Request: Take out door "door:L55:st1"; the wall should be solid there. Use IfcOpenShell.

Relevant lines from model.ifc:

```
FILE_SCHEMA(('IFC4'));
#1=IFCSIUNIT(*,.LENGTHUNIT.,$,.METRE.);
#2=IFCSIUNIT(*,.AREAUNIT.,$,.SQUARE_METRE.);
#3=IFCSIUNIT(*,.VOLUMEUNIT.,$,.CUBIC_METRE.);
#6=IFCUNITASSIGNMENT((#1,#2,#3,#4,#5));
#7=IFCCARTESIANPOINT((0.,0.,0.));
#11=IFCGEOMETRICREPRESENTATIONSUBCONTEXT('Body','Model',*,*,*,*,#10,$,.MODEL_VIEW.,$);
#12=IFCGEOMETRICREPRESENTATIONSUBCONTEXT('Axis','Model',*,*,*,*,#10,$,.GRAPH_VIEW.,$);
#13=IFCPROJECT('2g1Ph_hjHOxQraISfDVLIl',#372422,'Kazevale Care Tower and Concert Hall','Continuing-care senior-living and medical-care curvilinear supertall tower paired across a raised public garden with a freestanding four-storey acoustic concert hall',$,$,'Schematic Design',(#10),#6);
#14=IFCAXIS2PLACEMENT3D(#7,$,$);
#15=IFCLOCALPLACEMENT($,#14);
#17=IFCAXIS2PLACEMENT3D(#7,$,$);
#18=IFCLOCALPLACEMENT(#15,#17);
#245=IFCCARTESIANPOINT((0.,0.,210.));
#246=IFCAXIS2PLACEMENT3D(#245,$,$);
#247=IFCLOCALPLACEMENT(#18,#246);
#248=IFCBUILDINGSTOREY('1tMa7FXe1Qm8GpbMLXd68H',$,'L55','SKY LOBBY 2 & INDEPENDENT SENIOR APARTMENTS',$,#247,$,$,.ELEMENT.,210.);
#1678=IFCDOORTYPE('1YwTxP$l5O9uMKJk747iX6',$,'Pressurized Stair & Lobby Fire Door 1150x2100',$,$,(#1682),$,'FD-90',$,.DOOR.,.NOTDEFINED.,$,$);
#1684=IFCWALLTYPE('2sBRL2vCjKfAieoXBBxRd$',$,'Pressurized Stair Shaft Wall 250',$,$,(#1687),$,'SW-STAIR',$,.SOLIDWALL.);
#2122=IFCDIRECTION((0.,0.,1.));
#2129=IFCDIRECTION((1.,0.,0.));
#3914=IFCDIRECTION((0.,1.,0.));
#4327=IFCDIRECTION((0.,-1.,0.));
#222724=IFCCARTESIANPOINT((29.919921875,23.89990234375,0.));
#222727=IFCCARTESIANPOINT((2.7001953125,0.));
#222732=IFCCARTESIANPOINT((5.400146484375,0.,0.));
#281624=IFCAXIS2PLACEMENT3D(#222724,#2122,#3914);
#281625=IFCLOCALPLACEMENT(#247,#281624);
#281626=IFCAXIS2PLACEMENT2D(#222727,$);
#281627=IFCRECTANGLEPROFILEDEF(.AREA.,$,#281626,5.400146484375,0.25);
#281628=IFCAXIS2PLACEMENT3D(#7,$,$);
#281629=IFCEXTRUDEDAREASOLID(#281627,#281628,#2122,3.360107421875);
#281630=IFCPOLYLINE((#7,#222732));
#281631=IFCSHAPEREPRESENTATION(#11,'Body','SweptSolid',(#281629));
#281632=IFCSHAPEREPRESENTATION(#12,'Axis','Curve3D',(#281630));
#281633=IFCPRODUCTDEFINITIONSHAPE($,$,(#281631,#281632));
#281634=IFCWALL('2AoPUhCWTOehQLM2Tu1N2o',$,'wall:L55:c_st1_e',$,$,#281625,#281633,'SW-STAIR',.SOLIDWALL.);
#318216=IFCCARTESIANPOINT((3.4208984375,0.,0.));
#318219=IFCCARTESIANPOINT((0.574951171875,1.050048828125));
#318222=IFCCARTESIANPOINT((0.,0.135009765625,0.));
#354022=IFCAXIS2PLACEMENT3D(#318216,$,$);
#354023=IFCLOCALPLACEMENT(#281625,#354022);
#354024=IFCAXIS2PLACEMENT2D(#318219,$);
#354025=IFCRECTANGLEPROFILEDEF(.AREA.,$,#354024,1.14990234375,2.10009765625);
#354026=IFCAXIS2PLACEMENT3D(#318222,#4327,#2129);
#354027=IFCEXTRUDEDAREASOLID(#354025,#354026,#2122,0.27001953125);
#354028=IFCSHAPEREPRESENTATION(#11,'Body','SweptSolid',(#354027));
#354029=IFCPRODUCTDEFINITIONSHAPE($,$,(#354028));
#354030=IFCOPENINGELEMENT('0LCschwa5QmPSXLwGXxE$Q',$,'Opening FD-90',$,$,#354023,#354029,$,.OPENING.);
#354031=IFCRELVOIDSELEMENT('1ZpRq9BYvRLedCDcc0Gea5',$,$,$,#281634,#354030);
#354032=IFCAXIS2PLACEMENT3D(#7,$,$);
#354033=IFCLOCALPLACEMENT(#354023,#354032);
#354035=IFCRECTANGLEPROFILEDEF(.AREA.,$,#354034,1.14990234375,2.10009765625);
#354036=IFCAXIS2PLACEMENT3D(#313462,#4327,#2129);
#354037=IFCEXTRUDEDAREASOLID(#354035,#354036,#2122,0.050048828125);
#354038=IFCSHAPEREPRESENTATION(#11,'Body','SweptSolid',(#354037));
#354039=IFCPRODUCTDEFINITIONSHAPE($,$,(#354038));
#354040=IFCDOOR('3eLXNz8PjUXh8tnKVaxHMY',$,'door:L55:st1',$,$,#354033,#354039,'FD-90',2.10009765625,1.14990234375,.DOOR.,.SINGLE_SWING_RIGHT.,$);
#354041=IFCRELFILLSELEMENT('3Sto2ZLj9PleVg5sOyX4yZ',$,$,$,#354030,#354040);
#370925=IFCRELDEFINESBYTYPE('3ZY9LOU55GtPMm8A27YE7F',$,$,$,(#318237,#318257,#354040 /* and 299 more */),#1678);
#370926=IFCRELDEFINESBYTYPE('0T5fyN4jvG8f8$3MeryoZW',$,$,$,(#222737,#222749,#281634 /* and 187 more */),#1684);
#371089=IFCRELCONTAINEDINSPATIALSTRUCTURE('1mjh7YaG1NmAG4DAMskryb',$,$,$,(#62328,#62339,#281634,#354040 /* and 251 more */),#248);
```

```python
import ifcopenshell
import ifcopenshell.api.feature
import ifcopenshell.api.root
import ifcopenshell.geom
import ifcopenshell.util.shape

model = ifcopenshell.open("model.ifc")
settings = ifcopenshell.geom.settings()


def volume(element):
    """Net volume in cubic metres, openings subtracted."""
    shape = ifcopenshell.geom.create_shape(settings, element)
    return ifcopenshell.util.shape.get_volume(shape.geometry)


door = model.by_guid("3eLXNz8PjUXh8tnKVaxHMY")
opening = door.FillsVoids[0].RelatingOpeningElement
wall = opening.VoidsElements[0].RelatingBuildingElement
before = volume(wall)

ifcopenshell.api.root.remove_product(model, product=door)
ifcopenshell.api.feature.remove_feature(model, feature=opening)

after = volume(wall)

print(f"wall volume {before:.3f} -> {after:.3f} m3")

model.write("model_updated.ifc")
```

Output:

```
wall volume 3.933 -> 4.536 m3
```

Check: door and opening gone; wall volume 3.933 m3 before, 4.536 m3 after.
